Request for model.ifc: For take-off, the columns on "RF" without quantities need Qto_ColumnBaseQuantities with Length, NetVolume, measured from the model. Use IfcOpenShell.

First a look at what the model holds.

```python
import ifcopenshell
import ifcopenshell.util.element
import ifcopenshell.util.unit

model = ifcopenshell.open("model.ifc")
print(model.schema)
for unit_type in ("LENGTHUNIT", "AREAUNIT", "VOLUMEUNIT"):
    print(unit_type, ifcopenshell.util.unit.calculate_unit_scale(model, unit_type))
storey = next(s for s in model.by_type("IfcBuildingStorey") if s.Name == "RF")
columns = [e for e in ifcopenshell.util.element.get_decomposition(storey) if e.is_a("IfcColumn")]
for e in sorted(columns, key=lambda e: e.id()):
    print(e.id(), e.is_a(), e.Name, list(ifcopenshell.util.element.get_psets(e, qtos_only=True)), sep=" | ")
```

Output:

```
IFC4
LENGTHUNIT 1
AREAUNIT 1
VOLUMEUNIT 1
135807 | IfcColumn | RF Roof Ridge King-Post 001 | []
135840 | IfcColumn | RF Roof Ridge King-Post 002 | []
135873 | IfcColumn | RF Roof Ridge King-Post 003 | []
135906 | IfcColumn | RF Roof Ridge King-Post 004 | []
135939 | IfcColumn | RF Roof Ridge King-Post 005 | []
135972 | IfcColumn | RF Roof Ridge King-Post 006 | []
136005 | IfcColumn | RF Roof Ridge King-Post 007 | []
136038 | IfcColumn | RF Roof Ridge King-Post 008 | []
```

```python
import ifcopenshell
import ifcopenshell.api.pset
import ifcopenshell.geom
import ifcopenshell.util.element
import ifcopenshell.util.shape
import ifcopenshell.util.unit

model = ifcopenshell.open("model.ifc")
unit_scale = ifcopenshell.util.unit.calculate_unit_scale(model)
volume_scale = ifcopenshell.util.unit.calculate_unit_scale(model, "VOLUMEUNIT")
settings = ifcopenshell.geom.settings()

storey = next(s for s in model.by_type("IfcBuildingStorey") if s.Name == "RF")
columns = [e for e in ifcopenshell.util.element.get_decomposition(storey) if e.is_a("IfcColumn")]

for e in sorted(columns, key=lambda e: e.id()):
    if ifcopenshell.util.element.get_psets(e, qtos_only=True, should_inherit=False):
        continue
    # Geometry comes back in metres, in the element's own axes.
    shape = ifcopenshell.geom.create_shape(settings, e)
    values = {
        "Length": ifcopenshell.util.shape.get_z(shape.geometry) / unit_scale,
        "NetVolume": ifcopenshell.util.shape.get_volume(shape.geometry) / volume_scale,
    }
    qto = ifcopenshell.api.pset.add_qto(model, product=e, name="Qto_ColumnBaseQuantities")
    ifcopenshell.api.pset.edit_qto(model, qto=qto, properties=values)
    print(e.id(), {k: round(v, 3) for k, v in values.items()})

model.write("model_updated.ifc")
```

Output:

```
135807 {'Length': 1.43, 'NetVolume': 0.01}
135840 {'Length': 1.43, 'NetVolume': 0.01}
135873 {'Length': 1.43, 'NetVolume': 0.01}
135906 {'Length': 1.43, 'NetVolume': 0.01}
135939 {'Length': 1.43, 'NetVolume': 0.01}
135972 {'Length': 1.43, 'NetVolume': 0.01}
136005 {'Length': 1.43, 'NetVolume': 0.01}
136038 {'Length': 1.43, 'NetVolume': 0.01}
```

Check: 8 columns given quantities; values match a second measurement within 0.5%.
